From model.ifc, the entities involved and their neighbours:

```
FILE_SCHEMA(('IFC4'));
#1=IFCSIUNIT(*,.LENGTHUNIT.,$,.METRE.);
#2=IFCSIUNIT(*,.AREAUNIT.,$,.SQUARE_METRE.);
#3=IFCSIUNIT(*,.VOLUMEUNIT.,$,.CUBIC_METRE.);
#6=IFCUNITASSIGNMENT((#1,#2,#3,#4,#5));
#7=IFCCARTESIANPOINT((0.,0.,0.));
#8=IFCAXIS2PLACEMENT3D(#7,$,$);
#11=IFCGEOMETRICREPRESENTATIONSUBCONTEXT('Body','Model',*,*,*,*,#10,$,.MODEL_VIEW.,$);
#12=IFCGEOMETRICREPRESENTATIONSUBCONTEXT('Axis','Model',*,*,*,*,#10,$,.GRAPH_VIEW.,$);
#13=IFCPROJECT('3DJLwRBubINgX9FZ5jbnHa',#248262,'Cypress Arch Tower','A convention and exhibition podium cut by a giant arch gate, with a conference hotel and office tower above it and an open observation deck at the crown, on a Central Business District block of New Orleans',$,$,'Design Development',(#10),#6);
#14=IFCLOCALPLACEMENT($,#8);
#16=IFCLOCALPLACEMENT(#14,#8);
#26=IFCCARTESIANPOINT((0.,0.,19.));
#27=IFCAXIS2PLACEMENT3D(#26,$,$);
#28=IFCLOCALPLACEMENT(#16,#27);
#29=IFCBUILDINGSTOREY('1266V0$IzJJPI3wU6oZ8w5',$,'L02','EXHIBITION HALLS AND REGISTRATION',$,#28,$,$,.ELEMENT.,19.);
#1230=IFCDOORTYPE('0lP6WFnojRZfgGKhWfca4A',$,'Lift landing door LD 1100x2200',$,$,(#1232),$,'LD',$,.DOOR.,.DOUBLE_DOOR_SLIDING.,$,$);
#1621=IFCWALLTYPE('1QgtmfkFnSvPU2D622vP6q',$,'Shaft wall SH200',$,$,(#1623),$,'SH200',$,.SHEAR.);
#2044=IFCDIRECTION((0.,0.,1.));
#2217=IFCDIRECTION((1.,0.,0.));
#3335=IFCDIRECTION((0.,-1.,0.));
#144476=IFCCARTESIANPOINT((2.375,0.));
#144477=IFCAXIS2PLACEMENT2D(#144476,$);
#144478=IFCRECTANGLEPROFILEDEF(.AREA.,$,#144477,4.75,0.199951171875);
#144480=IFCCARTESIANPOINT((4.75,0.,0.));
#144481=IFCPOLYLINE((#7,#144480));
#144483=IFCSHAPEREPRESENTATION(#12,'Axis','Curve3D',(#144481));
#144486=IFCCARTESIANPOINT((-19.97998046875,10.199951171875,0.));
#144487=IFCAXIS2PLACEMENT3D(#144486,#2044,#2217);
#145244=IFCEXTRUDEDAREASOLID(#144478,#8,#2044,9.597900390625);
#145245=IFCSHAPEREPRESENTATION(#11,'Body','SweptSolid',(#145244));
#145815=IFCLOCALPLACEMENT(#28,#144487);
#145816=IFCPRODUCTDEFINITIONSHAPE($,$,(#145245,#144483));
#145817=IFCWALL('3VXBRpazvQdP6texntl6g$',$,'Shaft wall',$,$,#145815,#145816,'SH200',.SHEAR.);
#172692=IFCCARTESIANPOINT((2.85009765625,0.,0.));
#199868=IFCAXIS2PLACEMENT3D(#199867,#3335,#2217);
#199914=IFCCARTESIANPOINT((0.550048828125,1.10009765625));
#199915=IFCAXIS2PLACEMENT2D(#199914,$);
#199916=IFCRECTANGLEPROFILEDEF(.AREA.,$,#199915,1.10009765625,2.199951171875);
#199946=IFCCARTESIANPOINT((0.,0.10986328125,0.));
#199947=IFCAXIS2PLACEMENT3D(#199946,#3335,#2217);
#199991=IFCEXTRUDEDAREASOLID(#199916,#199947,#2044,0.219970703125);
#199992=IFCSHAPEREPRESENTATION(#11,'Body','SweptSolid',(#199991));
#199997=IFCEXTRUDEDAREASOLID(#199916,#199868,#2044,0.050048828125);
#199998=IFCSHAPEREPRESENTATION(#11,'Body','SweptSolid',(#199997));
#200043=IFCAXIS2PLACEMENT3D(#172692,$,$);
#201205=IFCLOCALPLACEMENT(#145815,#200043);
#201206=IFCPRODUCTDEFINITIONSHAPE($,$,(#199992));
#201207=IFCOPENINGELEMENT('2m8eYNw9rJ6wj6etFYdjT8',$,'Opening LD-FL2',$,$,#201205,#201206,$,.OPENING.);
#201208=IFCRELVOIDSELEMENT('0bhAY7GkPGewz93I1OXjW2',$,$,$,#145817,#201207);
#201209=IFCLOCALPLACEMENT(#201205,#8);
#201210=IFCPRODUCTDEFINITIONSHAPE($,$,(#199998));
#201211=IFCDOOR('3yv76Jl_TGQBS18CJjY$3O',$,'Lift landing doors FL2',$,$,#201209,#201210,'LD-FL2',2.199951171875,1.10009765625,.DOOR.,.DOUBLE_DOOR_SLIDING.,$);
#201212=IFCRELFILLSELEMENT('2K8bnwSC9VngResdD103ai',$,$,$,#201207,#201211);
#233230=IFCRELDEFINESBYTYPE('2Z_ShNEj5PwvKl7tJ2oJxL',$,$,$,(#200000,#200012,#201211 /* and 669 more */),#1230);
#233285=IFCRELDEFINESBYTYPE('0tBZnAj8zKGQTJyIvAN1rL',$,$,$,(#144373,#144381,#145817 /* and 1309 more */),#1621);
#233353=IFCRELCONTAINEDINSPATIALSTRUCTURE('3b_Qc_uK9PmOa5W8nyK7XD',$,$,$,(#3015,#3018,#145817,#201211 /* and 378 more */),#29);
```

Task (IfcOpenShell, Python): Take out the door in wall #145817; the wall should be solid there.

```python
import ifcopenshell
import ifcopenshell.api.feature
import ifcopenshell.api.root
import ifcopenshell.geom
import ifcopenshell.util.shape

model = ifcopenshell.open("model.ifc")
settings = ifcopenshell.geom.settings()


def volume(element):
    """Net volume in cubic metres, openings subtracted."""
    shape = ifcopenshell.geom.create_shape(settings, element)
    return ifcopenshell.util.shape.get_volume(shape.geometry)


door = model.by_guid("3yv76Jl_TGQBS18CJjY$3O")
opening = door.FillsVoids[0].RelatingOpeningElement
wall = opening.VoidsElements[0].RelatingBuildingElement
before = volume(wall)

ifcopenshell.api.root.remove_product(model, product=door)
ifcopenshell.api.feature.remove_feature(model, feature=opening)

after = volume(wall)

print(f"wall volume {before:.3f} -> {after:.3f} m3")

model.write("model_rev.ifc")
```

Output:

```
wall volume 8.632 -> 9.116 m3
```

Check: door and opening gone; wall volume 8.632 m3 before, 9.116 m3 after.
